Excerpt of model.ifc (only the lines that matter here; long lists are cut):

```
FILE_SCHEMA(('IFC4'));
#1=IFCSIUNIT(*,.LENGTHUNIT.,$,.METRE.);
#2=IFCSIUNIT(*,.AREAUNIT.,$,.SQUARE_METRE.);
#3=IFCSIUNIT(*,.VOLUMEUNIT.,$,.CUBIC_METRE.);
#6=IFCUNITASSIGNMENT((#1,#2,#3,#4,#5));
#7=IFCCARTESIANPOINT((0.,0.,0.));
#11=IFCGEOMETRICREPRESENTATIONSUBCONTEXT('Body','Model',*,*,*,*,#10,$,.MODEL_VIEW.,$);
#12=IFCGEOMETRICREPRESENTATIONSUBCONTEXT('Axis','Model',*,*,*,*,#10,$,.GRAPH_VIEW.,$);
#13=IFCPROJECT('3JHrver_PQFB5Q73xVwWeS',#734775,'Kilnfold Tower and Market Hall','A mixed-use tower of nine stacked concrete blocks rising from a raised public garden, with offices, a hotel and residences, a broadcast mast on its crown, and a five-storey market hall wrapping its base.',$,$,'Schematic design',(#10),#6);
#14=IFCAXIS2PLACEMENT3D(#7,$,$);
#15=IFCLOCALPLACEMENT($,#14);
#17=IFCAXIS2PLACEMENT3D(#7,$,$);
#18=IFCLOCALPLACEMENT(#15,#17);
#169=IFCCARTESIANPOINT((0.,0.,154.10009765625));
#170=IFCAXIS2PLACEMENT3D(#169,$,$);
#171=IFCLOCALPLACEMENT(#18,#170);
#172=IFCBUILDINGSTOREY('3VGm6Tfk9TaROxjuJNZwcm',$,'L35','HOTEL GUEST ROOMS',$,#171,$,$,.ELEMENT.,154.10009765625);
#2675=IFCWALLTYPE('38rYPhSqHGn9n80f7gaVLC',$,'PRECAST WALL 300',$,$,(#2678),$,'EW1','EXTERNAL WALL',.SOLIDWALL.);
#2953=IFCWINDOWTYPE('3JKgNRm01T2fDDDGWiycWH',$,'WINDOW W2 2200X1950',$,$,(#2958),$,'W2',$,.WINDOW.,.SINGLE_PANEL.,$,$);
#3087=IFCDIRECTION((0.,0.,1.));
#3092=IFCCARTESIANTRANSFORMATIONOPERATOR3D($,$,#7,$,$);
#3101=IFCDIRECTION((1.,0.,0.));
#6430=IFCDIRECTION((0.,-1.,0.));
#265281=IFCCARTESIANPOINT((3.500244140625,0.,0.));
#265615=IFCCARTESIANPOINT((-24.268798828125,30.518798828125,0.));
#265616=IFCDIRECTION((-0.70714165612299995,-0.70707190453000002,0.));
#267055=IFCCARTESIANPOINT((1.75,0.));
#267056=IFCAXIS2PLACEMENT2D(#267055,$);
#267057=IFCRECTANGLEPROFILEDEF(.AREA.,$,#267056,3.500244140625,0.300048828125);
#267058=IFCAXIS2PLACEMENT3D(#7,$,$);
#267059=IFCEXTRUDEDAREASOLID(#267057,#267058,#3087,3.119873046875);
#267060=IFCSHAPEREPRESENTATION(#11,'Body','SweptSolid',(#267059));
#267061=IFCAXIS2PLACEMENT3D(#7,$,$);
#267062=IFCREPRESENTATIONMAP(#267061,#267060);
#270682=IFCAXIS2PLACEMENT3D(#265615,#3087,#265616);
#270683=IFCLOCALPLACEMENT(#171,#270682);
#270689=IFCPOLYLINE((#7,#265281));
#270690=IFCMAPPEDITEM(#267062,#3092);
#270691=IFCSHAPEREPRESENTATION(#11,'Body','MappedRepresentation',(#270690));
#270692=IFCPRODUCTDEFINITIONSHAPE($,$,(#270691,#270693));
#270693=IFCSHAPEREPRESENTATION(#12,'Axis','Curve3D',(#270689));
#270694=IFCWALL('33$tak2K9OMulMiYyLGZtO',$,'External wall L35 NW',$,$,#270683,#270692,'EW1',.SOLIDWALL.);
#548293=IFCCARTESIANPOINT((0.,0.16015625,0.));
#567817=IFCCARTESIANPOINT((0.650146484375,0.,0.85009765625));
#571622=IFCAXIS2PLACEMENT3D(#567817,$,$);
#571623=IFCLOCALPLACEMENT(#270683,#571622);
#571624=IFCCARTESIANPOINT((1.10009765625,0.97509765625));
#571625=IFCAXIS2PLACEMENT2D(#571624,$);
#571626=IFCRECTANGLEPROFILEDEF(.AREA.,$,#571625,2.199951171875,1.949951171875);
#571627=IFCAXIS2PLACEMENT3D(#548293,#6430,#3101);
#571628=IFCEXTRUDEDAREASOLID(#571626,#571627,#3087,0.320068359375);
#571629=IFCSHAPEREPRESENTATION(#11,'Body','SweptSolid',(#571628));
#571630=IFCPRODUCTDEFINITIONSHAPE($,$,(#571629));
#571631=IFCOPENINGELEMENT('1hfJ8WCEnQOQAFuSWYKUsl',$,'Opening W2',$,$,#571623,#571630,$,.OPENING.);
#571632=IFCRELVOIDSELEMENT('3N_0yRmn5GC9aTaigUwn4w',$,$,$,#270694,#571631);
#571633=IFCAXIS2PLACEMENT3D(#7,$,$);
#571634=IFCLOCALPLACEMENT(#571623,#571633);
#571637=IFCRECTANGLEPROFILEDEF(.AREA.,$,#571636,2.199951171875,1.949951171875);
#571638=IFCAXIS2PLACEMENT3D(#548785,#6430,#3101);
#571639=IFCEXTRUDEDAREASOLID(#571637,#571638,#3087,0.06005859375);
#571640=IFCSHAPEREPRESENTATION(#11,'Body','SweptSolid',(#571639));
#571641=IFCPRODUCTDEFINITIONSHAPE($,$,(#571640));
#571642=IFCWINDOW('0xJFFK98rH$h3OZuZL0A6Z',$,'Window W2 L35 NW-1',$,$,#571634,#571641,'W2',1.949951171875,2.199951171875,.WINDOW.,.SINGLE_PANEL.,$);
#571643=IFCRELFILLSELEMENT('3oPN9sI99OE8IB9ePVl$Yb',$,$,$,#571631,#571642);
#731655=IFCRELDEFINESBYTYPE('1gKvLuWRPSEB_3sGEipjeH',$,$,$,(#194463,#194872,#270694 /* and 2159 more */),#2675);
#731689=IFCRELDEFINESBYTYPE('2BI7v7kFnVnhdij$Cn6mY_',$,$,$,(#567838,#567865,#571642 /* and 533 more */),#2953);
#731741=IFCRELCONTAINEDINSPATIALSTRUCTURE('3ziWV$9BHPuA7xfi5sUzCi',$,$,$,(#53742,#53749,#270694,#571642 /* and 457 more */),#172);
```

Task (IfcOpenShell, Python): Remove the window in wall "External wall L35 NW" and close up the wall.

```python
import ifcopenshell
import ifcopenshell.api.feature
import ifcopenshell.api.root
import ifcopenshell.geom
import ifcopenshell.util.shape

model = ifcopenshell.open("model.ifc")
settings = ifcopenshell.geom.settings()


def volume(element):
    """Net volume in cubic metres, openings subtracted."""
    shape = ifcopenshell.geom.create_shape(settings, element)
    return ifcopenshell.util.shape.get_volume(shape.geometry)


window = model.by_id(571642)
opening = window.FillsVoids[0].RelatingOpeningElement
wall = opening.VoidsElements[0].RelatingBuildingElement
before = volume(wall)

ifcopenshell.api.root.remove_product(model, product=window)
ifcopenshell.api.feature.remove_feature(model, feature=opening)

after = volume(wall)

print(f"wall volume {before:.3f} -> {after:.3f} m3")

model.write("model_edited.ifc")
```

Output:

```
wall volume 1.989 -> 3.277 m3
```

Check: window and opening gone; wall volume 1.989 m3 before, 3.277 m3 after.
